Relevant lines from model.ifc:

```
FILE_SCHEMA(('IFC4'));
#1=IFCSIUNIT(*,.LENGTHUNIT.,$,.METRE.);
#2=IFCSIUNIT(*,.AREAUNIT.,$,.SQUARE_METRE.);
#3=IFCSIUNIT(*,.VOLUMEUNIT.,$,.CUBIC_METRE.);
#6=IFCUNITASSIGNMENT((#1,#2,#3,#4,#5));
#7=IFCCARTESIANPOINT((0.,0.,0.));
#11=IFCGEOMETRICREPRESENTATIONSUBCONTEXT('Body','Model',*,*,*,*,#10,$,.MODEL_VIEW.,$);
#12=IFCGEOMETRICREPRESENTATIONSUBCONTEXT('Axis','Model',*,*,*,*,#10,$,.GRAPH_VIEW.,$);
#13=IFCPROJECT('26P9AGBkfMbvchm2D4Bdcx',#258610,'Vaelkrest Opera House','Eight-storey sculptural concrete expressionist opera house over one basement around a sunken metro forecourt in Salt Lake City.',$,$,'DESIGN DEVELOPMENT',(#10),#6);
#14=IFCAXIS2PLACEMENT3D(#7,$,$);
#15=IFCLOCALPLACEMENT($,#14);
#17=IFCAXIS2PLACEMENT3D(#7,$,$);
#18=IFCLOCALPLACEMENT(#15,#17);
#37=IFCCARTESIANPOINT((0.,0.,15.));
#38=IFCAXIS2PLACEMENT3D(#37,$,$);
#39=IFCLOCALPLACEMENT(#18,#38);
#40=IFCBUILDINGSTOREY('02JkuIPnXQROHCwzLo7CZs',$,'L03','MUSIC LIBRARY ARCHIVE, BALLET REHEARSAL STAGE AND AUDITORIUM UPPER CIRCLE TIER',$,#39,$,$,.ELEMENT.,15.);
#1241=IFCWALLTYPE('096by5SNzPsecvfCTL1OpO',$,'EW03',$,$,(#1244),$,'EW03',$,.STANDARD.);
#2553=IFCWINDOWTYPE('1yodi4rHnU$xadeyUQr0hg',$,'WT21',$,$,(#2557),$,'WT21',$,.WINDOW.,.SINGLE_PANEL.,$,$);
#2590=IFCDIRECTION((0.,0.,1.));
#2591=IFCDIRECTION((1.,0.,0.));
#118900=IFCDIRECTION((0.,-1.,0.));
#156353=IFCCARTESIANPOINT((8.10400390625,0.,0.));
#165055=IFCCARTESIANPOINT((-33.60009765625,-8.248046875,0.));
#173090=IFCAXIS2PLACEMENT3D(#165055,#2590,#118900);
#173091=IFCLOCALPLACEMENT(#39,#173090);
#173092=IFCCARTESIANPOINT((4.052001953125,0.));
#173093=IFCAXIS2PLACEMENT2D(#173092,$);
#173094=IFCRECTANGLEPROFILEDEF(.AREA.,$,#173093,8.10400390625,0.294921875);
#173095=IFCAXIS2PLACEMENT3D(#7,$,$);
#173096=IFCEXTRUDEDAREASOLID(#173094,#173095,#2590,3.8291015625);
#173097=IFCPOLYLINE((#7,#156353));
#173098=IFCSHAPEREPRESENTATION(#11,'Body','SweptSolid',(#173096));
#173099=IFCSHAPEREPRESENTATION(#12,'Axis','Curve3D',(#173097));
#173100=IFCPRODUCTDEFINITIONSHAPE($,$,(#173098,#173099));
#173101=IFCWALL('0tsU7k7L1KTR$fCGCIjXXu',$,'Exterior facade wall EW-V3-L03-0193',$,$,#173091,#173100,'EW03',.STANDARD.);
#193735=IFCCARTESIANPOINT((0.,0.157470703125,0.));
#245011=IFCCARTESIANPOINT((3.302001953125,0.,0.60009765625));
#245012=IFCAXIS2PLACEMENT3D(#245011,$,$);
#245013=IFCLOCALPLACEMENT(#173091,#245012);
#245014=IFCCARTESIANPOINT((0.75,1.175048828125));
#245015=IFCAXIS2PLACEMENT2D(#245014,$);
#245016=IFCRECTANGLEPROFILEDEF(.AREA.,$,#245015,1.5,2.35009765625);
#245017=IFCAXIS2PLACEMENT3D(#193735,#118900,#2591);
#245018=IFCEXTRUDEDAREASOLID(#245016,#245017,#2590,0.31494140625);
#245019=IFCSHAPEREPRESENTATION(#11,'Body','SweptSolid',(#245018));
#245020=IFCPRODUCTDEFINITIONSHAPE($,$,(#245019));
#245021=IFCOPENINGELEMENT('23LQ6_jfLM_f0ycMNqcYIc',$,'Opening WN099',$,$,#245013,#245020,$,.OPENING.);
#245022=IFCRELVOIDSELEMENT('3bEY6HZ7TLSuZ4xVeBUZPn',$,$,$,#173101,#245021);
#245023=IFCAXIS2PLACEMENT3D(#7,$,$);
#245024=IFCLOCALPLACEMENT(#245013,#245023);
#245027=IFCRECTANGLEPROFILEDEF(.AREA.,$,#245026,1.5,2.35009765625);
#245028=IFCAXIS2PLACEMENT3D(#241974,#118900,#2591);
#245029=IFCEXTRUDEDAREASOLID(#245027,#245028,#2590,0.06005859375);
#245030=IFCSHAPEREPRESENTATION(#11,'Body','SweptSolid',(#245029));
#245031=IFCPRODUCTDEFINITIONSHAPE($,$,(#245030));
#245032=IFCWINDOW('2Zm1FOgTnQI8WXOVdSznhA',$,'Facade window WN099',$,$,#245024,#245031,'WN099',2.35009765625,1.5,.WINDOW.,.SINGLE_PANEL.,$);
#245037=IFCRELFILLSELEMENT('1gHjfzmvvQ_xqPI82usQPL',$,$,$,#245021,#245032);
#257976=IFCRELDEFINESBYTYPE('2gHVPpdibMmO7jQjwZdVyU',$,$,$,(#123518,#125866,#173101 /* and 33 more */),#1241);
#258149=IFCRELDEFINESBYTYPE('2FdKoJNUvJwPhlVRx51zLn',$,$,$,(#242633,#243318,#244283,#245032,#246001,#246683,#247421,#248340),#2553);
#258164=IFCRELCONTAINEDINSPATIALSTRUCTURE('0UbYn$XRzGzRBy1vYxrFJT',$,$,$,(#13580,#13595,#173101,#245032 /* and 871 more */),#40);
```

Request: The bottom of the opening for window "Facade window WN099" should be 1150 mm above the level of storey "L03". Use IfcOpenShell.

```python
import numpy as np
import ifcopenshell
import ifcopenshell.api.geometry
import ifcopenshell.geom
import ifcopenshell.util.element
import ifcopenshell.util.placement
import ifcopenshell.util.shape
import ifcopenshell.util.unit

model = ifcopenshell.open("model.ifc")
unit_scale = ifcopenshell.util.unit.calculate_unit_scale(model)

window = model.by_guid("2Zm1FOgTnQI8WXOVdSznhA")
opening = window.FillsVoids[0].RelatingOpeningElement
storey = ifcopenshell.util.element.get_container(window, ifc_class="IfcBuildingStorey")
level = ifcopenshell.util.placement.get_local_placement(storey.ObjectPlacement)[2, 3]

# The opening's origin need not be at the sill, so measure its lowest point.
shape = ifcopenshell.geom.create_shape(ifcopenshell.geom.settings(), opening)
bottom = ifcopenshell.util.shape.get_shape_bottom_elevation(shape, shape.geometry) / unit_scale
dz = level + 1.15 / unit_scale - bottom

shift = np.array([0.0, 0.0, dz])
# The window is placed relative to its opening, so it follows when the opening moves.
matrix = ifcopenshell.util.placement.get_local_placement(opening.ObjectPlacement)
matrix[:3, 3] += shift
ifcopenshell.api.geometry.edit_object_placement(
    model, product=opening, matrix=matrix, is_si=False, should_transform_children=True
)

print(f"moved by {dz * unit_scale:+.3f} m")

model.write("model_rev.ifc")
```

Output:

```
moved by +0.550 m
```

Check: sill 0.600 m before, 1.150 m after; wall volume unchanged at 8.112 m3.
